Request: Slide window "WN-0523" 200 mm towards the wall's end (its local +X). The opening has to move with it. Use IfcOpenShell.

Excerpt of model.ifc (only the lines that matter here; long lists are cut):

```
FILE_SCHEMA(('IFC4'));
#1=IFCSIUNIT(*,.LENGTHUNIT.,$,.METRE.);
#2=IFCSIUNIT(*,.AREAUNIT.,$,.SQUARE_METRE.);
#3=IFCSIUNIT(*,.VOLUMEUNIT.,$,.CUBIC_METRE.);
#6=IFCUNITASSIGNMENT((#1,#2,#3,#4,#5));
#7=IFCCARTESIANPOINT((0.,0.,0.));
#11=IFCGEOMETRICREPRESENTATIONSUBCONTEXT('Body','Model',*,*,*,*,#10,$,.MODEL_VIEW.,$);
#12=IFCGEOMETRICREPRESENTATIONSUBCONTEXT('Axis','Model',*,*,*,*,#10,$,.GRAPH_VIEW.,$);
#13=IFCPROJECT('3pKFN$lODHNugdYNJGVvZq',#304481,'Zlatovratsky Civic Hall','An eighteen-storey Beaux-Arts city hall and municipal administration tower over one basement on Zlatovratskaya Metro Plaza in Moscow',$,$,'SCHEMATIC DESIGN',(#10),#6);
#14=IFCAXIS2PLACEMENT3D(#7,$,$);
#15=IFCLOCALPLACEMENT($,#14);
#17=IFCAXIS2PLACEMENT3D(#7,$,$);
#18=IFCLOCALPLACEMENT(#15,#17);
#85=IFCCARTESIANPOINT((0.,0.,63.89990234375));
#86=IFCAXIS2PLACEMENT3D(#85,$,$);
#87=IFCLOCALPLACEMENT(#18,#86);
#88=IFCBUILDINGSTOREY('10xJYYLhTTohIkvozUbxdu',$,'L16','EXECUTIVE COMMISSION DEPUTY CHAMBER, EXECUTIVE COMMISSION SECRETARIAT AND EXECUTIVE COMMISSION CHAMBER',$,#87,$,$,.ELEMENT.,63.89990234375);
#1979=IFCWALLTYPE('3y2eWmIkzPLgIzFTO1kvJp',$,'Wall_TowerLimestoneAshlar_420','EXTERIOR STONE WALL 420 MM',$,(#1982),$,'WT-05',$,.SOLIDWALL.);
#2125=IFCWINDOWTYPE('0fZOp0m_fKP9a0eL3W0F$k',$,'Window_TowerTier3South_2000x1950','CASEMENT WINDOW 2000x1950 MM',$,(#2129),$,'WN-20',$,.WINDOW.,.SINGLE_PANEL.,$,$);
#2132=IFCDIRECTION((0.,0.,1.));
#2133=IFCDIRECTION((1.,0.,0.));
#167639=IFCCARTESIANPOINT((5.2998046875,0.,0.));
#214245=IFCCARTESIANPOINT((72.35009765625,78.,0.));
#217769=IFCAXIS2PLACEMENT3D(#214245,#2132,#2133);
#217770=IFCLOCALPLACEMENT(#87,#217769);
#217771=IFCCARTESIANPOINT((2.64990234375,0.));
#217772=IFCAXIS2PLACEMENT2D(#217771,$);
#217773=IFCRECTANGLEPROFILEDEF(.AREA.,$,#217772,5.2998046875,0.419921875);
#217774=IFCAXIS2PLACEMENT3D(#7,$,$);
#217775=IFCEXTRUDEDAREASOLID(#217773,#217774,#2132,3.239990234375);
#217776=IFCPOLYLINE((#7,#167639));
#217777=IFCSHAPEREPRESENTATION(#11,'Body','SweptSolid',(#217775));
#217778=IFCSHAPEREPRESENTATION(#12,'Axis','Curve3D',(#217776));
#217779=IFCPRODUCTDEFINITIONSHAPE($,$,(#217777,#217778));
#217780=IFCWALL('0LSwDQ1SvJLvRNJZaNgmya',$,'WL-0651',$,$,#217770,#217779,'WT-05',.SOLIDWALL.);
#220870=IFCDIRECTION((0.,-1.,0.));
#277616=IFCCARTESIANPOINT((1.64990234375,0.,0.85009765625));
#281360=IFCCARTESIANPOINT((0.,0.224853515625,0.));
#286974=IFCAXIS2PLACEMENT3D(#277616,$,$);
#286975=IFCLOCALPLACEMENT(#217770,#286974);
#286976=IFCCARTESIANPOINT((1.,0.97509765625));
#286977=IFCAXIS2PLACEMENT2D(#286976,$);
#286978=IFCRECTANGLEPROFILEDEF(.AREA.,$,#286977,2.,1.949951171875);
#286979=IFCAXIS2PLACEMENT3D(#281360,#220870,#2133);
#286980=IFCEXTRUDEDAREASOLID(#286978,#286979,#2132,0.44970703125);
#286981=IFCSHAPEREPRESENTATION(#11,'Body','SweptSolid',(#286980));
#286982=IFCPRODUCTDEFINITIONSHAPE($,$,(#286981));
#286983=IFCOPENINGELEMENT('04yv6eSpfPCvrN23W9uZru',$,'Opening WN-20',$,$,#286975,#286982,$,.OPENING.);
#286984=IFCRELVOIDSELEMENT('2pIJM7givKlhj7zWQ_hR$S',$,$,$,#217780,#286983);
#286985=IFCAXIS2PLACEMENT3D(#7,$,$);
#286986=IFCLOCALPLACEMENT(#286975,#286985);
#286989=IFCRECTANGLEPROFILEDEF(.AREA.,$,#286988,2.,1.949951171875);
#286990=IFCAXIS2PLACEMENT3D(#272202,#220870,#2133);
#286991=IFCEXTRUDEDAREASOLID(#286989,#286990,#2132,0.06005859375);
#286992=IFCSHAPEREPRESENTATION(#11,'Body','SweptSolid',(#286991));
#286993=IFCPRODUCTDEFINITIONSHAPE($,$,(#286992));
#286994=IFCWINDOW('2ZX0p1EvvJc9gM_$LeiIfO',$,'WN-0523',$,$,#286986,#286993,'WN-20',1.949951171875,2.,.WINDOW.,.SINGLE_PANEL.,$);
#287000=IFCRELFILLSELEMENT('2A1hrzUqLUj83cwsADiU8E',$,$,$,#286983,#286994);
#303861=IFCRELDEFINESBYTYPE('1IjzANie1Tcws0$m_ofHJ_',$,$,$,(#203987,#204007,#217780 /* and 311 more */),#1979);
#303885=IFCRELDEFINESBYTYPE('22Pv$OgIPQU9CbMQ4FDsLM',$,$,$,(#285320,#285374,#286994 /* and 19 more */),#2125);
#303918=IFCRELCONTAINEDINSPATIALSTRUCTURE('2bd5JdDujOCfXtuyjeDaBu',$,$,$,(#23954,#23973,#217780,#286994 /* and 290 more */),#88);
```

```python
import ifcopenshell
import ifcopenshell.api.geometry
import ifcopenshell.util.placement

model = ifcopenshell.open("model.ifc")

window = model.by_guid("2ZX0p1EvvJc9gM_$LeiIfO")
opening = window.FillsVoids[0].RelatingOpeningElement
wall = opening.VoidsElements[0].RelatingBuildingElement

wall_matrix = ifcopenshell.util.placement.get_local_placement(wall.ObjectPlacement)
shift = wall_matrix[:3, 0] * 0.2
before = ifcopenshell.util.placement.get_local_placement(window.ObjectPlacement)[:3, 3].copy()

# The window is placed relative to its opening, so it follows when the opening moves.
matrix = ifcopenshell.util.placement.get_local_placement(opening.ObjectPlacement)
matrix[:3, 3] += shift
ifcopenshell.api.geometry.edit_object_placement(
    model, product=opening, matrix=matrix, is_si=False, should_transform_children=True
)

after = ifcopenshell.util.placement.get_local_placement(window.ObjectPlacement)[:3, 3]
print("window moved by", (after - before).round(3) + 0.0)

model.write("model_v2.ifc")
```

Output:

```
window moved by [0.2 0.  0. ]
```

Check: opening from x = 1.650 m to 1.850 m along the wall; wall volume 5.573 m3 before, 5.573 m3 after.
